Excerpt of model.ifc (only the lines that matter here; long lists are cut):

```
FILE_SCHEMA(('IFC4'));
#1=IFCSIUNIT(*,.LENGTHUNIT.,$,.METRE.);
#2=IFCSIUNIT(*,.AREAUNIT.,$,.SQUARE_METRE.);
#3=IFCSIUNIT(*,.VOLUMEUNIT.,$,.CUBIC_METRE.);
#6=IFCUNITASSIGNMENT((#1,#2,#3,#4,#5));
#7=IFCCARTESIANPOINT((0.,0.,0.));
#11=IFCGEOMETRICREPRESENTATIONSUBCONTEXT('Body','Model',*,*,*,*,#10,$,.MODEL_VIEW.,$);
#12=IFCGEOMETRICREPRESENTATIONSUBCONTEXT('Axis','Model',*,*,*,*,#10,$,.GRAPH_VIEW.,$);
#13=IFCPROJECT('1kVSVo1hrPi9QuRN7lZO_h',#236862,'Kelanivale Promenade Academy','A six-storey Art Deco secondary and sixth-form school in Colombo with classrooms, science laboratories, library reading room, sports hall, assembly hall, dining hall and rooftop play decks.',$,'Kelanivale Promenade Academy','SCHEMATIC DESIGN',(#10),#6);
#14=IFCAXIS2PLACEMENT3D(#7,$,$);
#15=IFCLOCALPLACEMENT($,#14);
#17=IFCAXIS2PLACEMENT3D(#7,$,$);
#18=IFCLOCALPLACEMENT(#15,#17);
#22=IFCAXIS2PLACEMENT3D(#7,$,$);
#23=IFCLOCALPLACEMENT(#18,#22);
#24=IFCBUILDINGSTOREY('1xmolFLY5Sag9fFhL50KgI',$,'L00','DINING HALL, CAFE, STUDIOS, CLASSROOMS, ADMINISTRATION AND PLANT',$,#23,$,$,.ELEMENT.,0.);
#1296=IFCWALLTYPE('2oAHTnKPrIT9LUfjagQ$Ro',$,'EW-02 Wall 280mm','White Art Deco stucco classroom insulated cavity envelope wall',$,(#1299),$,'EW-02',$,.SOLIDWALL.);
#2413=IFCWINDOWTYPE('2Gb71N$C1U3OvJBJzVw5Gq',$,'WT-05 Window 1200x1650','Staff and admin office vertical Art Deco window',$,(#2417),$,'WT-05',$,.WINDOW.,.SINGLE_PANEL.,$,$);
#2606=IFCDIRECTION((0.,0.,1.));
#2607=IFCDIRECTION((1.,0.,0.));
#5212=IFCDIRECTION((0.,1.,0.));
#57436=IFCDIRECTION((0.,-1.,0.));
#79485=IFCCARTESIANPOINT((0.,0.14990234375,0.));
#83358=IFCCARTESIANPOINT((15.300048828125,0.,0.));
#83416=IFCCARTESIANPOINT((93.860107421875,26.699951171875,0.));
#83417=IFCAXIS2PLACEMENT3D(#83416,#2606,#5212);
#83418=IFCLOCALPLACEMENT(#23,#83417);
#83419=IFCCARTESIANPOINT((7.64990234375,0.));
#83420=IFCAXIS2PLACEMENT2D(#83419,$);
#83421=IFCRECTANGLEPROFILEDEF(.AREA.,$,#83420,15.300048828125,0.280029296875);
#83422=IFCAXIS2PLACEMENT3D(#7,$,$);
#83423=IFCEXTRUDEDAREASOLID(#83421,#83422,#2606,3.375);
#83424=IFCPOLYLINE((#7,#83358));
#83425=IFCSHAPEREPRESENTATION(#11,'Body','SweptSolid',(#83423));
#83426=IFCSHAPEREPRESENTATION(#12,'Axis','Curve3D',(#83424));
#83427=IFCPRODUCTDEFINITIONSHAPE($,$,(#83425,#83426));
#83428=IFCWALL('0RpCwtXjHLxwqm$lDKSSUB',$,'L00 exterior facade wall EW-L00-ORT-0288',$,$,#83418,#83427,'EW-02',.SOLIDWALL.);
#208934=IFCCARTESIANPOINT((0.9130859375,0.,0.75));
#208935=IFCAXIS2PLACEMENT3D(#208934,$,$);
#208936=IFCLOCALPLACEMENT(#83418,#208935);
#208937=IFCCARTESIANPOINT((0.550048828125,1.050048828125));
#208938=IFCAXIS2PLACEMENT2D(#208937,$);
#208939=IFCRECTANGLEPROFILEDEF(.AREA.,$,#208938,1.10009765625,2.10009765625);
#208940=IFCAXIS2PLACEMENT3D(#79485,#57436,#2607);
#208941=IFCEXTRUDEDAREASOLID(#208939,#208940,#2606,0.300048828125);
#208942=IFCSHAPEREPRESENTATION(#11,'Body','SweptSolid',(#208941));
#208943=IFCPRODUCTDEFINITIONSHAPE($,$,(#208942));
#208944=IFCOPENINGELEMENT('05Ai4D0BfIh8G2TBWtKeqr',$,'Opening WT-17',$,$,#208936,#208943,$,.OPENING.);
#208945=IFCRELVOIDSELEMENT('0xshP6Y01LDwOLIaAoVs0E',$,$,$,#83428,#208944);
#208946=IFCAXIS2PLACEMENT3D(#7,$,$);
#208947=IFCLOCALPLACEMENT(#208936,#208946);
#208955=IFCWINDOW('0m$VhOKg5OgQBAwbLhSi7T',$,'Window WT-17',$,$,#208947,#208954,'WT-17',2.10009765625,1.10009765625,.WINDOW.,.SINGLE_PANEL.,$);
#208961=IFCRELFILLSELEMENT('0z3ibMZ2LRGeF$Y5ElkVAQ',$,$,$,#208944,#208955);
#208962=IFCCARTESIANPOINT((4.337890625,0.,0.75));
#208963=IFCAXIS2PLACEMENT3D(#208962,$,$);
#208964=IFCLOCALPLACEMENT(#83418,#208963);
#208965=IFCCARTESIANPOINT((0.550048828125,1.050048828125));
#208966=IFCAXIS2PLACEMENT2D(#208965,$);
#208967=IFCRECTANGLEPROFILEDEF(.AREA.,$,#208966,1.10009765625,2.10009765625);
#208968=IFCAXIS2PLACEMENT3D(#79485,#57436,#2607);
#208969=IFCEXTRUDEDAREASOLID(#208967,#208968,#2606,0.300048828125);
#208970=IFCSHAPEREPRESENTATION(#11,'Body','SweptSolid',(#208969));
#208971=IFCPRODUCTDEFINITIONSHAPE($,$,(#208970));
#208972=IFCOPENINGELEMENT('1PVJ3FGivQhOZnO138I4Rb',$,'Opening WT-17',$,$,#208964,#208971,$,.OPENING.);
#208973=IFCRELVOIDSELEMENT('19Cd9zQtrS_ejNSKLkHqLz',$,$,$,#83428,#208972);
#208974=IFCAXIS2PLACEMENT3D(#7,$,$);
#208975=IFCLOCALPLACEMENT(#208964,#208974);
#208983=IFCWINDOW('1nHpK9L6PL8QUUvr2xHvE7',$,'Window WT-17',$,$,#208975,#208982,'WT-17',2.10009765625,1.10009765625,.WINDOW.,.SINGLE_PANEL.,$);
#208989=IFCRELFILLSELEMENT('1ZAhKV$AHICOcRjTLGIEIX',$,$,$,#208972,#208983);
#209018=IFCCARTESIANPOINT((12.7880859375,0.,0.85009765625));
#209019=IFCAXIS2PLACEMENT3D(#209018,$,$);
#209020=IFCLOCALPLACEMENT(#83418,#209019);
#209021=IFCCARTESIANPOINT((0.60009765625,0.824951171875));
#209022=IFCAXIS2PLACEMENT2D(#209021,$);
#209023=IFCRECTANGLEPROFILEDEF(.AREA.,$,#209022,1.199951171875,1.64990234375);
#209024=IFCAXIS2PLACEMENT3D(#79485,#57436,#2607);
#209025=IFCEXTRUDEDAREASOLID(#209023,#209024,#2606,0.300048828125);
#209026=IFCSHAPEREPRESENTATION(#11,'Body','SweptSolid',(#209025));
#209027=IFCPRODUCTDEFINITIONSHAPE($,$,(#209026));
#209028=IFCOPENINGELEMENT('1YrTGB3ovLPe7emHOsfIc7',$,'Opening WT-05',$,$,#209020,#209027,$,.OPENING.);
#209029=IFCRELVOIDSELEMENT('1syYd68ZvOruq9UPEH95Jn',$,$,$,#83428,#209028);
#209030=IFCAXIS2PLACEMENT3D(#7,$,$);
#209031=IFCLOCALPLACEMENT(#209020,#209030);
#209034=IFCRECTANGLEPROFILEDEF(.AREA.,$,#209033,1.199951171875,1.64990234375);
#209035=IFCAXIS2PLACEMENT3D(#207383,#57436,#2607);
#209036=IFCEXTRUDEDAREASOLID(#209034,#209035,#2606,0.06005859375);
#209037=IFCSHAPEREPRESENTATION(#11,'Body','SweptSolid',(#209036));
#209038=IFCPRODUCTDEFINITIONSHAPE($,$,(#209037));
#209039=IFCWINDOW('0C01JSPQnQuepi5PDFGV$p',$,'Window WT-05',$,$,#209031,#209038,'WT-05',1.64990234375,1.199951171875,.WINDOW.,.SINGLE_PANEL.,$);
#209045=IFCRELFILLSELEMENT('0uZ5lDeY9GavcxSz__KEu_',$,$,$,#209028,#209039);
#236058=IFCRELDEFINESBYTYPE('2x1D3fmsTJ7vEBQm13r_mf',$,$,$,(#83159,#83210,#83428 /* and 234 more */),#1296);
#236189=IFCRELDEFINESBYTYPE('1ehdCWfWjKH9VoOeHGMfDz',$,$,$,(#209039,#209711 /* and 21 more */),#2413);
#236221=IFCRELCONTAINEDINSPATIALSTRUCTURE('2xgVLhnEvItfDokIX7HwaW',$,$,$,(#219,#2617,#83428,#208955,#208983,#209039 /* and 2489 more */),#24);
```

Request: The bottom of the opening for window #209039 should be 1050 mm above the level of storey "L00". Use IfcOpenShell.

```python
import numpy as np
import ifcopenshell
import ifcopenshell.api.geometry
import ifcopenshell.geom
import ifcopenshell.util.element
import ifcopenshell.util.placement
import ifcopenshell.util.shape
import ifcopenshell.util.unit

model = ifcopenshell.open("model.ifc")
unit_scale = ifcopenshell.util.unit.calculate_unit_scale(model)

window = model.by_guid("0C01JSPQnQuepi5PDFGV$p")
opening = window.FillsVoids[0].RelatingOpeningElement
storey = ifcopenshell.util.element.get_container(window, ifc_class="IfcBuildingStorey")
level = ifcopenshell.util.placement.get_local_placement(storey.ObjectPlacement)[2, 3]

# The opening's origin need not be at the sill, so measure its lowest point.
shape = ifcopenshell.geom.create_shape(ifcopenshell.geom.settings(), opening)
bottom = ifcopenshell.util.shape.get_shape_bottom_elevation(shape, shape.geometry) / unit_scale
dz = level + 1.05 / unit_scale - bottom

shift = np.array([0.0, 0.0, dz])
# The window is placed relative to its opening, so it follows when the opening moves.
matrix = ifcopenshell.util.placement.get_local_placement(opening.ObjectPlacement)
matrix[:3, 3] += shift
ifcopenshell.api.geometry.edit_object_placement(
    model, product=opening, matrix=matrix, is_si=False, should_transform_children=True
)

print(f"moved by {dz * unit_scale:+.3f} m")

model.write("model_edited.ifc")
```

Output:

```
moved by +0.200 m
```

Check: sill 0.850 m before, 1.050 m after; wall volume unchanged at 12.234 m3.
